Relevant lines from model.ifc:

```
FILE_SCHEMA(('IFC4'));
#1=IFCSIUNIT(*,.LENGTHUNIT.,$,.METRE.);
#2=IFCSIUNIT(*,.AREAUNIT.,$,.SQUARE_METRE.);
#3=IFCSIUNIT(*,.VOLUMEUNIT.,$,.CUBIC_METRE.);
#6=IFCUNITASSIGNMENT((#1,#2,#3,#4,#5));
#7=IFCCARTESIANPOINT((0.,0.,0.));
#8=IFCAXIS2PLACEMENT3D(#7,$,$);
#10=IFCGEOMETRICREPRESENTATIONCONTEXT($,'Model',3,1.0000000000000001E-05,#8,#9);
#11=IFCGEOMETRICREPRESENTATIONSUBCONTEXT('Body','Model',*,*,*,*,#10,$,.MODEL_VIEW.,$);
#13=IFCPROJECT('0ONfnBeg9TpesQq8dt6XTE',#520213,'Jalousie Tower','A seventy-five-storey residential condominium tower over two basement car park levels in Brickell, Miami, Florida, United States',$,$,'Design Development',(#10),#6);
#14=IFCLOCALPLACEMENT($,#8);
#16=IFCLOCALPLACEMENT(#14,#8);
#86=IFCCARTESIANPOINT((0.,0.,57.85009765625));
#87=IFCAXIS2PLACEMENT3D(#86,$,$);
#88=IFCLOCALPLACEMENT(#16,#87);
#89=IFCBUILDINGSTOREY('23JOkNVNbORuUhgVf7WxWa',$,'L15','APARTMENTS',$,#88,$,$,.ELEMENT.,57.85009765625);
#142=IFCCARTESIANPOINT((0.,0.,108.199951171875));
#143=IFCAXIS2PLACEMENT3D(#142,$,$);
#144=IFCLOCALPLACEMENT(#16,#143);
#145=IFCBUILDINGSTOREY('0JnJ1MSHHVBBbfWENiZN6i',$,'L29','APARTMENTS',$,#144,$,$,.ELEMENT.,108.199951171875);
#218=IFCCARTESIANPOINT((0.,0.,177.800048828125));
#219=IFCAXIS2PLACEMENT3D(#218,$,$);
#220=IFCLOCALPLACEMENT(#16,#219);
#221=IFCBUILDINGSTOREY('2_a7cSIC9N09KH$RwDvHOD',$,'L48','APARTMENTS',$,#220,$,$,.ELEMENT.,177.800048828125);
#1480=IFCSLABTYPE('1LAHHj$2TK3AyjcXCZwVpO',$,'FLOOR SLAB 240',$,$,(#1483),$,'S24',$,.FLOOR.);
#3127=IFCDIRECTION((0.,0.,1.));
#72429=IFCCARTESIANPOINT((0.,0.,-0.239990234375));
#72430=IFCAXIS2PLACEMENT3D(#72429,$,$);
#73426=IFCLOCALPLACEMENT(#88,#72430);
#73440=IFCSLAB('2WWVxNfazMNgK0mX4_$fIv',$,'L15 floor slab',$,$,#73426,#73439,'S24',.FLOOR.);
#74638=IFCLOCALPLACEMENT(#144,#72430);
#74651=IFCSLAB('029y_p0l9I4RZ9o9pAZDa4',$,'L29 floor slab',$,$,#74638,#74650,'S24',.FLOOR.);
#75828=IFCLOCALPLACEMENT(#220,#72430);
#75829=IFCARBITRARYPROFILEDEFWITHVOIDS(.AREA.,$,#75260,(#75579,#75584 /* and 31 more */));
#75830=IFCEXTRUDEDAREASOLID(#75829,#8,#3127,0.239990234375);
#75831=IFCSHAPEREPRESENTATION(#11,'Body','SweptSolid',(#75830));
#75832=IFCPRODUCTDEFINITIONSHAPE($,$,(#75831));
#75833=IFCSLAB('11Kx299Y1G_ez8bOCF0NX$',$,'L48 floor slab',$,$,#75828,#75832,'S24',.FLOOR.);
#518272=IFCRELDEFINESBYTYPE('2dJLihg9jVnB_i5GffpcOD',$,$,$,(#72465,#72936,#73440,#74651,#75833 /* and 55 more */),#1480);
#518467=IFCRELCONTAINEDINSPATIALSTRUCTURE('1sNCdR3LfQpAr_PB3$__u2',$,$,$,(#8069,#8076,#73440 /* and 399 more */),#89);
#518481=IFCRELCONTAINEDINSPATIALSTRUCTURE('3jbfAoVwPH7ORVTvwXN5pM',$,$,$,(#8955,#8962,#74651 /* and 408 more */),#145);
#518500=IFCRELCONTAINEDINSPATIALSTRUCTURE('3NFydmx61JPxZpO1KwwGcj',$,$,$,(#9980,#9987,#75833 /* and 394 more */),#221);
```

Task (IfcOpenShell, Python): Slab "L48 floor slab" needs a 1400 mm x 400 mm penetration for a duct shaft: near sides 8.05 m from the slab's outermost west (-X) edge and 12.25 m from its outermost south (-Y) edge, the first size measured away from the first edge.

```python
import numpy as np
import ifcopenshell
import ifcopenshell.api.feature
import ifcopenshell.api.geometry
import ifcopenshell.api.root
import ifcopenshell.geom
import ifcopenshell.util.placement
import ifcopenshell.util.representation
import ifcopenshell.util.shape
import ifcopenshell.util.unit

model = ifcopenshell.open("model.ifc")
unit_scale = ifcopenshell.util.unit.calculate_unit_scale(model)
settings = ifcopenshell.geom.settings()


def volume(element):
    """Net volume in cubic metres, openings subtracted."""
    shape = ifcopenshell.geom.create_shape(settings, element)
    return ifcopenshell.util.shape.get_volume(shape.geometry)


slab = model.by_guid("11Kx299Y1G_ez8bOCF0NX$")
before = volume(slab)

# Extent in the slab's own axes, in metres. The edges named are its -X and -Y sides.
slab_shape = ifcopenshell.geom.create_shape(settings, slab)
vertices = ifcopenshell.util.shape.get_vertices(slab_shape.geometry)
x_min, y_min, bottom = vertices.min(axis=0)
top = vertices[:, 2].max()

opening = ifcopenshell.api.root.create_entity(model, ifc_class="IfcOpeningElement", name="Duct shaft opening", predefined_type="OPENING")
context = ifcopenshell.util.representation.get_context(model, "Model", "Body", "MODEL_VIEW")
width, depth = 1.4, 0.4
outline = [(0.0, 0.0), (width, 0.0), (width, depth), (0.0, depth), (0.0, 0.0)]
# Overshoot both faces by 50 mm so the cut is clean.
shape = ifcopenshell.api.geometry.add_slab_representation(
    model, context=context, depth=top - bottom + 0.1, polyline=outline
)
ifcopenshell.api.geometry.assign_representation(model, product=opening, representation=shape)

matrix = ifcopenshell.util.placement.get_local_placement(slab.ObjectPlacement)
matrix[:, 3] = matrix @ np.append(np.array([x_min + 8.05, y_min + 12.25, bottom - 0.05]) / unit_scale, 1.0)
ifcopenshell.api.geometry.edit_object_placement(model, product=opening, matrix=matrix, is_si=False)
ifcopenshell.api.feature.add_feature(model, feature=opening, element=slab)

after = volume(slab)

print(f"slab volume {before:.3f} -> {after:.3f} m3")

model.write("model_v2.ifc")
```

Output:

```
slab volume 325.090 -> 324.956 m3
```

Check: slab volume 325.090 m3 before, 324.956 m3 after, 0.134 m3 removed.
